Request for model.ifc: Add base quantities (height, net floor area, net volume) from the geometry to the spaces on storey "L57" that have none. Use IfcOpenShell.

First a look at what the model holds.

```python
import ifcopenshell
import ifcopenshell.util.element
import ifcopenshell.util.unit

model = ifcopenshell.open("model.ifc")
print(model.schema)
for unit_type in ("LENGTHUNIT", "AREAUNIT", "VOLUMEUNIT"):
    print(unit_type, ifcopenshell.util.unit.calculate_unit_scale(model, unit_type))
storey = next(s for s in model.by_type("IfcBuildingStorey") if s.Name == "L57")
spaces = [e for e in ifcopenshell.util.element.get_decomposition(storey) if e.is_a("IfcSpace")]
for e in sorted(spaces, key=lambda e: e.id()):
    print(e.id(), e.is_a(), e.Name, list(ifcopenshell.util.element.get_psets(e, qtos_only=True)), sep=" | ")
```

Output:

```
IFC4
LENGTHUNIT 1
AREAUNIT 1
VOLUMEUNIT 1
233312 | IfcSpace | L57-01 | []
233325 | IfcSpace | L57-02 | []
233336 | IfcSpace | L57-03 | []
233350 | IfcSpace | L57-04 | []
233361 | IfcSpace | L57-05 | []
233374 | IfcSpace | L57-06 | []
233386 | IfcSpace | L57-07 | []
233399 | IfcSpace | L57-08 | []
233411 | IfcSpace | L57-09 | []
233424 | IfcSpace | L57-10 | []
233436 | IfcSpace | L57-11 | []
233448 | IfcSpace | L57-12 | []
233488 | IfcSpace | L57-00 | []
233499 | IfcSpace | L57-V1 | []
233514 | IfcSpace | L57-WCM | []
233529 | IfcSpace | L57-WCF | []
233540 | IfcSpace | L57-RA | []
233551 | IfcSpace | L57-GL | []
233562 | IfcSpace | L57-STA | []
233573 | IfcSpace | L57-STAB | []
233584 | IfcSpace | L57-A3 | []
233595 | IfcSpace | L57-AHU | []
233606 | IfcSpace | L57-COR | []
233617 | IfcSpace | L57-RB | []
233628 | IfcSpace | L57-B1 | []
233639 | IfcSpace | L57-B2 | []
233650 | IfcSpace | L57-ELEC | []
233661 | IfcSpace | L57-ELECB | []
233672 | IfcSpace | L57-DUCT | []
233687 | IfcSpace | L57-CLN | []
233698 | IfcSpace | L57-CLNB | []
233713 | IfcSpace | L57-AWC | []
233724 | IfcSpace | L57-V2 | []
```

```python
import ifcopenshell
import ifcopenshell.api.pset
import ifcopenshell.geom
import ifcopenshell.util.element
import ifcopenshell.util.shape
import ifcopenshell.util.unit

model = ifcopenshell.open("model.ifc")
unit_scale = ifcopenshell.util.unit.calculate_unit_scale(model)
area_scale = ifcopenshell.util.unit.calculate_unit_scale(model, "AREAUNIT")
volume_scale = ifcopenshell.util.unit.calculate_unit_scale(model, "VOLUMEUNIT")
settings = ifcopenshell.geom.settings()

storey = next(s for s in model.by_type("IfcBuildingStorey") if s.Name == "L57")
spaces = [e for e in ifcopenshell.util.element.get_decomposition(storey) if e.is_a("IfcSpace")]

for e in sorted(spaces, key=lambda e: e.id()):
    if ifcopenshell.util.element.get_psets(e, qtos_only=True, should_inherit=False):
        continue
    # Geometry comes back in metres, in the element's own axes.
    shape = ifcopenshell.geom.create_shape(settings, e)
    values = {
        "Height": ifcopenshell.util.shape.get_z(shape.geometry) / unit_scale,
        "NetFloorArea": ifcopenshell.util.shape.get_footprint_area(shape.geometry) / area_scale,
        "NetVolume": ifcopenshell.util.shape.get_volume(shape.geometry) / volume_scale,
    }
    qto = ifcopenshell.api.pset.add_qto(model, product=e, name="Qto_SpaceBaseQuantities")
    ifcopenshell.api.pset.edit_qto(model, qto=qto, properties=values)
    print(e.id(), {k: round(v, 3) for k, v in values.items()})

model.write("model-out.ifc")
```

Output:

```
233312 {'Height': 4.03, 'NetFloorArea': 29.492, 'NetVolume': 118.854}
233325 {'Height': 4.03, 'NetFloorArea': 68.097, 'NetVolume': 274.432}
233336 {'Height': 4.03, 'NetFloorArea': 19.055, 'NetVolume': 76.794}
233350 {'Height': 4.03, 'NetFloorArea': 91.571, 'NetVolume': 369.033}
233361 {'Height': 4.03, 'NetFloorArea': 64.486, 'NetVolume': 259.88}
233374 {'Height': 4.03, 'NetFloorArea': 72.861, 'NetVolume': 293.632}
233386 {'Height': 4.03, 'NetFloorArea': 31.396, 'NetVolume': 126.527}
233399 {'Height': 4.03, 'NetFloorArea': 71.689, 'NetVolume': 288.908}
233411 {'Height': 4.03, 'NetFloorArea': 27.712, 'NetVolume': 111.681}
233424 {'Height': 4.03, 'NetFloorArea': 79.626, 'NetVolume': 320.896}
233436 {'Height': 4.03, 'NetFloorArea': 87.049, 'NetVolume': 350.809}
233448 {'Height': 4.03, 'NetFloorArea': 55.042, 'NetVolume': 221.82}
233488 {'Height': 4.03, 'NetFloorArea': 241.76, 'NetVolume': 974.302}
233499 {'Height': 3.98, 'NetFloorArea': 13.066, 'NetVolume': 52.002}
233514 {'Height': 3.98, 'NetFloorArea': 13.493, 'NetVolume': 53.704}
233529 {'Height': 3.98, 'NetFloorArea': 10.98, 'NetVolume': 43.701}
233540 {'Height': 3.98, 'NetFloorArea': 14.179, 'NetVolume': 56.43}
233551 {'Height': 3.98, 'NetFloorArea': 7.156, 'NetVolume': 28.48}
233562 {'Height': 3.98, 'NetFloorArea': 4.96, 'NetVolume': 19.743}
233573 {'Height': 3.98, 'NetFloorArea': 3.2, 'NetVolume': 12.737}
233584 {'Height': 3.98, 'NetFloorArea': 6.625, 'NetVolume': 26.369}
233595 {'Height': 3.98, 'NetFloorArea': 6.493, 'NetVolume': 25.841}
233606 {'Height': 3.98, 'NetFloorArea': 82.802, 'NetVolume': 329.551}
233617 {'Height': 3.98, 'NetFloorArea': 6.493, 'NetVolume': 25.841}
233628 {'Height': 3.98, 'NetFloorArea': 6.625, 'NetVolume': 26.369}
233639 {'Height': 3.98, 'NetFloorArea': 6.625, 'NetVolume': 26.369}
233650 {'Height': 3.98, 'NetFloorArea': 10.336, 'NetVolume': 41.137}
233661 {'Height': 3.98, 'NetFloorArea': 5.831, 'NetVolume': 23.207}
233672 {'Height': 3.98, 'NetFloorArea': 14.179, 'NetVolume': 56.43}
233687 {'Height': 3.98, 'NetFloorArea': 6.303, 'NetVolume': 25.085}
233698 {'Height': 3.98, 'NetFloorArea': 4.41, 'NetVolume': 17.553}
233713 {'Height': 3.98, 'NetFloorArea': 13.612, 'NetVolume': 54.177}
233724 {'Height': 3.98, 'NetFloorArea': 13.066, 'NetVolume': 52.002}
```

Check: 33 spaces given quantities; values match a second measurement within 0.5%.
